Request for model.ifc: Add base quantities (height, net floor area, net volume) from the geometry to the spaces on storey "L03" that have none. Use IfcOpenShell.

First a look at what the model holds.

```python
import ifcopenshell
import ifcopenshell.util.element
import ifcopenshell.util.unit

model = ifcopenshell.open("model.ifc")
print(model.schema)
for unit_type in ("LENGTHUNIT", "AREAUNIT", "VOLUMEUNIT"):
    print(unit_type, ifcopenshell.util.unit.calculate_unit_scale(model, unit_type))
storey = next(s for s in model.by_type("IfcBuildingStorey") if s.Name == "L03")
spaces = [e for e in ifcopenshell.util.element.get_decomposition(storey) if e.is_a("IfcSpace")]
for e in sorted(spaces, key=lambda e: e.id()):
    print(e.id(), e.is_a(), e.Name, list(ifcopenshell.util.element.get_psets(e, qtos_only=True)), sep=" | ")
```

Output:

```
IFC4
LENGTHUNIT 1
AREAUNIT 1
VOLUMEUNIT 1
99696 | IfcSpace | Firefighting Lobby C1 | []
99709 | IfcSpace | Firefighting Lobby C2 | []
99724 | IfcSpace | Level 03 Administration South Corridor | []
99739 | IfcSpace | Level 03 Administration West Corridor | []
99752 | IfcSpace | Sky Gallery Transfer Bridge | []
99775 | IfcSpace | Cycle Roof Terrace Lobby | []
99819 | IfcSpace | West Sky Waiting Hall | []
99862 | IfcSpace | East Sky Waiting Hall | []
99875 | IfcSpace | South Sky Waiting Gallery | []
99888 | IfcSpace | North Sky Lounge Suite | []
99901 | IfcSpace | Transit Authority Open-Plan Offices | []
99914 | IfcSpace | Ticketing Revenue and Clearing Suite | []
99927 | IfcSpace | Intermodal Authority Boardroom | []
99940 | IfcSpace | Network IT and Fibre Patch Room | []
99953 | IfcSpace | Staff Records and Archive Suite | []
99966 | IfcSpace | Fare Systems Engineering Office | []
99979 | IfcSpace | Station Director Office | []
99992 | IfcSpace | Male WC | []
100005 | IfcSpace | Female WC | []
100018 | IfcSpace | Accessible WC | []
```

```python
import ifcopenshell
import ifcopenshell.api.pset
import ifcopenshell.geom
import ifcopenshell.util.element
import ifcopenshell.util.shape
import ifcopenshell.util.unit

model = ifcopenshell.open("model.ifc")
unit_scale = ifcopenshell.util.unit.calculate_unit_scale(model)
area_scale = ifcopenshell.util.unit.calculate_unit_scale(model, "AREAUNIT")
volume_scale = ifcopenshell.util.unit.calculate_unit_scale(model, "VOLUMEUNIT")
settings = ifcopenshell.geom.settings()

storey = next(s for s in model.by_type("IfcBuildingStorey") if s.Name == "L03")
spaces = [e for e in ifcopenshell.util.element.get_decomposition(storey) if e.is_a("IfcSpace")]

for e in sorted(spaces, key=lambda e: e.id()):
    if ifcopenshell.util.element.get_psets(e, qtos_only=True, should_inherit=False):
        continue
    # Geometry comes back in metres, in the element's own axes.
    shape = ifcopenshell.geom.create_shape(settings, e)
    values = {
        "Height": ifcopenshell.util.shape.get_z(shape.geometry) / unit_scale,
        "NetFloorArea": ifcopenshell.util.shape.get_footprint_area(shape.geometry) / area_scale,
        "NetVolume": ifcopenshell.util.shape.get_volume(shape.geometry) / volume_scale,
    }
    qto = ifcopenshell.api.pset.add_qto(model, product=e, name="Qto_SpaceBaseQuantities")
    ifcopenshell.api.pset.edit_qto(model, qto=qto, properties=values)
    print(e.id(), {k: round(v, 3) for k, v in values.items()})

model.write("model_rev.ifc")
```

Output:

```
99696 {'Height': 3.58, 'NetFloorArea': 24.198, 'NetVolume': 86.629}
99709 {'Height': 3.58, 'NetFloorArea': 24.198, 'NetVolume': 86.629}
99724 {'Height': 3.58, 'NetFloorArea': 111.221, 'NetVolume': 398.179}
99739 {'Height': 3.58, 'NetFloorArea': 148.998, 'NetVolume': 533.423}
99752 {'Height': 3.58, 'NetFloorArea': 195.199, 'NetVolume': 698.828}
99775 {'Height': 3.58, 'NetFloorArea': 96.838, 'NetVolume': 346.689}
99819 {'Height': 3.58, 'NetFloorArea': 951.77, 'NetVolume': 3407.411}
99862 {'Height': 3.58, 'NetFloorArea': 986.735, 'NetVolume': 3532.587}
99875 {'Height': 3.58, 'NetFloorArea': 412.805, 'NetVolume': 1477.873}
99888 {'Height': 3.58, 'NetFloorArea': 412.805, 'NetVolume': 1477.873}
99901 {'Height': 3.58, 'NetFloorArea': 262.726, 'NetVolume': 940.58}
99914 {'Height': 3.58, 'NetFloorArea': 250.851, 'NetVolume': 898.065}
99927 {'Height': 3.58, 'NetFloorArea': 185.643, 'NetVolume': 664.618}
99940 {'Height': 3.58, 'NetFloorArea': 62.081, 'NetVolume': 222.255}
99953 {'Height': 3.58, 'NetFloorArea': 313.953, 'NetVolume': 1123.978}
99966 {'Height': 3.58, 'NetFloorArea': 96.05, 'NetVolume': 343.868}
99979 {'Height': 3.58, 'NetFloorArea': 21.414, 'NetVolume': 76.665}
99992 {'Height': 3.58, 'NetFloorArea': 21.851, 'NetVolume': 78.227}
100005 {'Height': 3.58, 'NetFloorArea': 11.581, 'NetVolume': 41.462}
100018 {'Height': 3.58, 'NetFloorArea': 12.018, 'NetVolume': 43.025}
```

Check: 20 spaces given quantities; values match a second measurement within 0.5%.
